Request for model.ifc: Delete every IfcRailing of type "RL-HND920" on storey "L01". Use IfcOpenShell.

First a look at what the model holds.

```python
import ifcopenshell
import ifcopenshell.util.element

model = ifcopenshell.open("model.ifc")
print(model.schema)
storey = next(s for s in model.by_type("IfcBuildingStorey") if s.Name == "L01")
railings = [e for e in ifcopenshell.util.element.get_decomposition(storey) if e.is_a("IfcRailing")]
seen = {}
for e in railings:
    element_type = ifcopenshell.util.element.get_type(e)
    name = element_type.Name if element_type not in (None, e) else None
    seen[name] = seen.get(name, 0) + 1
for name, count in sorted(seen.items(), key=str):
    print(count, "x", name)
```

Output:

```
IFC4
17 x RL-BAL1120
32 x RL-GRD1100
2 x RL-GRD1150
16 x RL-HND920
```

```python
import ifcopenshell
import ifcopenshell.api.root
import ifcopenshell.util.element

model = ifcopenshell.open("model.ifc")

storey = next(s for s in model.by_type("IfcBuildingStorey") if s.Name == "L01")
railings = [e for e in ifcopenshell.util.element.get_decomposition(storey) if e.is_a("IfcRailing")]
targets = [e for e in railings if (t := ifcopenshell.util.element.get_type(e)) not in (None, e) and t.Name == "RL-HND920"]

for e in targets:
    ifcopenshell.api.root.remove_product(model, product=e)
print(len(targets), "removed")

model.write("model_v2.ifc")
```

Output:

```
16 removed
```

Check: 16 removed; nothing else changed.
